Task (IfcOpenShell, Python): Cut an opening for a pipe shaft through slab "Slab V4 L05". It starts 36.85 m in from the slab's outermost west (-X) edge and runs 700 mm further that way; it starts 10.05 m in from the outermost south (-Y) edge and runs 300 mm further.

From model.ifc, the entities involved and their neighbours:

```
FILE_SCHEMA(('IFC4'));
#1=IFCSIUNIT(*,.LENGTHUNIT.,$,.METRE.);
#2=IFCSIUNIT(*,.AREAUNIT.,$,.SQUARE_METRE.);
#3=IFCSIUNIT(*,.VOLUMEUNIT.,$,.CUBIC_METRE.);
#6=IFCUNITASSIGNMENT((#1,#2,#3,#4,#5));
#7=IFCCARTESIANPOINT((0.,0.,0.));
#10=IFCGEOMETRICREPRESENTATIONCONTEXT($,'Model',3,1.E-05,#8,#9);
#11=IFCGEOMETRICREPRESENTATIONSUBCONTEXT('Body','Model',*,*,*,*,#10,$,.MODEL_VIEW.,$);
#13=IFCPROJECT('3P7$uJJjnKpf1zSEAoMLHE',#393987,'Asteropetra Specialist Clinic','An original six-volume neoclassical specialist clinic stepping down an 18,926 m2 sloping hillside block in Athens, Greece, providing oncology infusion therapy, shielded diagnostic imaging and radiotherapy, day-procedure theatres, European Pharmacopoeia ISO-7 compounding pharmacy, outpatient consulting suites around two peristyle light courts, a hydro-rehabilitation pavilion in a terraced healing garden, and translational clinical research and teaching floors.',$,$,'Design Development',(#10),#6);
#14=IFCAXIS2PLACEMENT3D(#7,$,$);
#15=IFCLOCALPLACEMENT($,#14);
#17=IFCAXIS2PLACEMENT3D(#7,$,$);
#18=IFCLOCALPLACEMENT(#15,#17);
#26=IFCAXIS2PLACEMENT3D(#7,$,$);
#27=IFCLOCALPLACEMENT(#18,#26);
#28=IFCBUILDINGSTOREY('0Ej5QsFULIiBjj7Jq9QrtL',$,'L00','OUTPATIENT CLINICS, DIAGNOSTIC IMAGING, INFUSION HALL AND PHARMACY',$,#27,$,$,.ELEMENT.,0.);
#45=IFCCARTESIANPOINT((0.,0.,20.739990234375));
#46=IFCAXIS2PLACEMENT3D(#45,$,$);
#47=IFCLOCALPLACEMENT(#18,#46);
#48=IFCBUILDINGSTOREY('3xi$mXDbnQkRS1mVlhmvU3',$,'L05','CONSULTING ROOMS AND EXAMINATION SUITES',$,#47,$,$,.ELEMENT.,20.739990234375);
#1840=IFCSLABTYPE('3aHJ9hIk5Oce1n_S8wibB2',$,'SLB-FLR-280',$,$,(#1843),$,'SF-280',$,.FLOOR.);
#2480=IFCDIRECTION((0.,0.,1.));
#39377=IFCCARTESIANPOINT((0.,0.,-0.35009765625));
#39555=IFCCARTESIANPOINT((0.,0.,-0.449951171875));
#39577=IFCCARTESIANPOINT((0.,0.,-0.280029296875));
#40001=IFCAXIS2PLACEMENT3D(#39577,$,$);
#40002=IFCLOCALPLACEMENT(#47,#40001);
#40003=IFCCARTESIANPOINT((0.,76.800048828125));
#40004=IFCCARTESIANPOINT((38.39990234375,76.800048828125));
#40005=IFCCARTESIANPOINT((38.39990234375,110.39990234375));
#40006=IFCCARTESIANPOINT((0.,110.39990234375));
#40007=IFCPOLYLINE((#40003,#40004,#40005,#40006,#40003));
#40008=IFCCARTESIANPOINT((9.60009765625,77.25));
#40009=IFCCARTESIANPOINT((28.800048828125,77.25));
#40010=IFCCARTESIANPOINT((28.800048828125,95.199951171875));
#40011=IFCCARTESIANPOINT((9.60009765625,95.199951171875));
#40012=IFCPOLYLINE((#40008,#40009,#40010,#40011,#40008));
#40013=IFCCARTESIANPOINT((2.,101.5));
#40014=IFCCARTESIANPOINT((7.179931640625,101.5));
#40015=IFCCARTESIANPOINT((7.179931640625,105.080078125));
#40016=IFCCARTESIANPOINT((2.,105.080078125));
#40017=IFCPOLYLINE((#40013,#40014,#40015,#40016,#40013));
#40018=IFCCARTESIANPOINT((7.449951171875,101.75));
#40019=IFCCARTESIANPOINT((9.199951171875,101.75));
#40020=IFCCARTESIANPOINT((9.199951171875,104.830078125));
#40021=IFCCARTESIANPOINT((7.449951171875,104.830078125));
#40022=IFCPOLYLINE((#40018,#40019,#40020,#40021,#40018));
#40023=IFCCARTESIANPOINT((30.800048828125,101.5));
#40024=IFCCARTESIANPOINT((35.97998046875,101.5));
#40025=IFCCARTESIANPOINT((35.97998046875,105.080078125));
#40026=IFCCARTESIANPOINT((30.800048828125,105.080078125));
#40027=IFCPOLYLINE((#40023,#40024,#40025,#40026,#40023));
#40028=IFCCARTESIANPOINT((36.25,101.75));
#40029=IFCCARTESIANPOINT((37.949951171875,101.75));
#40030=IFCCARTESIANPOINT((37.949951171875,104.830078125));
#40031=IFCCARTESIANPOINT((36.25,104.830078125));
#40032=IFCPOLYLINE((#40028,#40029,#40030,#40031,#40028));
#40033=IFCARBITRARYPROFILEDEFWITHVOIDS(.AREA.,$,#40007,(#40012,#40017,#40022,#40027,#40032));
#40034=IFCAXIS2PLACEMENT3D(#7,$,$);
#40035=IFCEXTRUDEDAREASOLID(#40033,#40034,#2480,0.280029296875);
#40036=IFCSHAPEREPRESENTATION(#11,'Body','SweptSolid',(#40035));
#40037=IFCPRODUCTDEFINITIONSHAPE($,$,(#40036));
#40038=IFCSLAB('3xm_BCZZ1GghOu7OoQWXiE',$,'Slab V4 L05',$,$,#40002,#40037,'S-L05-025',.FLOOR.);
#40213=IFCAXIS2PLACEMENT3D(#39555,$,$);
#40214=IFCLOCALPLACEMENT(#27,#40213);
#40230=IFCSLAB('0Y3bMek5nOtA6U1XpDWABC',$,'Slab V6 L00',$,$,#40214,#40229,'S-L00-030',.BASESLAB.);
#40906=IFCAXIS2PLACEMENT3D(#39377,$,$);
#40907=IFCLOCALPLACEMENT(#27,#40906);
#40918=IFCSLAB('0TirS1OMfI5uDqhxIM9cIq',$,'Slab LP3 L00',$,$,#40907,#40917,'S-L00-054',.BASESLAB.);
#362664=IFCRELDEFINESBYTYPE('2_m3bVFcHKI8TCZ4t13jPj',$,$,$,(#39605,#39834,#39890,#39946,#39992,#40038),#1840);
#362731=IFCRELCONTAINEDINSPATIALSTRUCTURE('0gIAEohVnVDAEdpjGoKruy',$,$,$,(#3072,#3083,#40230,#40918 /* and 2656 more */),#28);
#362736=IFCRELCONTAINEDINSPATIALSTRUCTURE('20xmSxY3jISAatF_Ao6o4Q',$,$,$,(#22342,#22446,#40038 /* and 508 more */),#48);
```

```python
import numpy as np
import ifcopenshell
import ifcopenshell.api.feature
import ifcopenshell.api.geometry
import ifcopenshell.api.root
import ifcopenshell.geom
import ifcopenshell.util.placement
import ifcopenshell.util.representation
import ifcopenshell.util.shape
import ifcopenshell.util.unit

model = ifcopenshell.open("model.ifc")
unit_scale = ifcopenshell.util.unit.calculate_unit_scale(model)
settings = ifcopenshell.geom.settings()


def volume(element):
    """Net volume in cubic metres, openings subtracted."""
    shape = ifcopenshell.geom.create_shape(settings, element)
    return ifcopenshell.util.shape.get_volume(shape.geometry)


slab = model.by_guid("3xm_BCZZ1GghOu7OoQWXiE")
before = volume(slab)

# Extent in the slab's own axes, in metres. The edges named are its -X and -Y sides.
slab_shape = ifcopenshell.geom.create_shape(settings, slab)
vertices = ifcopenshell.util.shape.get_vertices(slab_shape.geometry)
x_min, y_min, bottom = vertices.min(axis=0)
top = vertices[:, 2].max()

opening = ifcopenshell.api.root.create_entity(model, ifc_class="IfcOpeningElement", name="Pipe shaft opening", predefined_type="OPENING")
context = ifcopenshell.util.representation.get_context(model, "Model", "Body", "MODEL_VIEW")
width, depth = 0.7, 0.3
outline = [(0.0, 0.0), (width, 0.0), (width, depth), (0.0, depth), (0.0, 0.0)]
# Overshoot both faces by 50 mm so the cut is clean.
shape = ifcopenshell.api.geometry.add_slab_representation(
    model, context=context, depth=top - bottom + 0.1, polyline=outline
)
ifcopenshell.api.geometry.assign_representation(model, product=opening, representation=shape)

matrix = ifcopenshell.util.placement.get_local_placement(slab.ObjectPlacement)
matrix[:, 3] = matrix @ np.append(np.array([x_min + 36.85, y_min + 10.05, bottom - 0.05]) / unit_scale, 1.0)
ifcopenshell.api.geometry.edit_object_placement(model, product=opening, matrix=matrix, is_si=False)
ifcopenshell.api.feature.add_feature(model, feature=opening, element=slab)

after = volume(slab)

print(f"slab volume {before:.3f} -> {after:.3f} m3")

model.write("model_updated.ifc")
```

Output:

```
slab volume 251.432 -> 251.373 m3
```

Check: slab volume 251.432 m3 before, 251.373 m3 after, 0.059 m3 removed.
